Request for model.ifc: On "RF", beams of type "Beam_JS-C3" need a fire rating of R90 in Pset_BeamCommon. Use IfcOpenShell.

First a look at what the model holds.

```python
import ifcopenshell
import ifcopenshell.util.element

model = ifcopenshell.open("model.ifc")
print(model.schema)
storey = next(s for s in model.by_type("IfcBuildingStorey") if s.Name == "RF")
beams = [e for e in ifcopenshell.util.element.get_decomposition(storey) if e.is_a("IfcBeam")]
seen = {}
for e in beams:
    element_type = ifcopenshell.util.element.get_type(e)
    key = (element_type.Name if element_type != e and element_type else None, ifcopenshell.util.element.get_pset(e, "Pset_BeamCommon", "FireRating"))
    seen[key] = seen.get(key, 0) + 1
for (name, value), count in sorted(seen.items(), key=str):
    print(count, "x", name, "|", value)
```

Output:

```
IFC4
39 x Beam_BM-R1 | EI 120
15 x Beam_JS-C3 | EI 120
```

```python
import ifcopenshell
import ifcopenshell.api.pset
import ifcopenshell.util.element

model = ifcopenshell.open("model.ifc")

storey = next(s for s in model.by_type("IfcBuildingStorey") if s.Name == "RF")
beams = [e for e in ifcopenshell.util.element.get_decomposition(storey) if e.is_a("IfcBeam")]

count = 0
for e in beams:
    element_type = ifcopenshell.util.element.get_type(e)
    if element_type in (None, e) or element_type.Name != "Beam_JS-C3":
        continue
    # add_pset returns the element's existing set when there is one.
    pset = ifcopenshell.api.pset.add_pset(model, product=e, name="Pset_BeamCommon")
    ifcopenshell.api.pset.edit_pset(model, pset=pset, properties={"FireRating": "R90"})
    count += 1

print(count, "beams updated")

model.write("model_v2.ifc")
```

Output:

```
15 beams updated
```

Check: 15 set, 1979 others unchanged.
